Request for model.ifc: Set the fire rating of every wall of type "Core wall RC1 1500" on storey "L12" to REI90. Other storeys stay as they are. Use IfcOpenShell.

First a look at what the model holds.

```python
import ifcopenshell
import ifcopenshell.util.element

model = ifcopenshell.open("model.ifc")
print(model.schema)
storey = next(s for s in model.by_type("IfcBuildingStorey") if s.Name == "L12")
walls = [e for e in ifcopenshell.util.element.get_decomposition(storey) if e.is_a("IfcWall")]
seen = {}
for e in walls:
    element_type = ifcopenshell.util.element.get_type(e)
    key = (element_type.Name if element_type != e and element_type else None, ifcopenshell.util.element.get_pset(e, "Pset_WallCommon", "FireRating"))
    seen[key] = seen.get(key, 0) + 1
for (name, value), count in sorted(seen.items(), key=str):
    print(count, "x", name, "|", value)
```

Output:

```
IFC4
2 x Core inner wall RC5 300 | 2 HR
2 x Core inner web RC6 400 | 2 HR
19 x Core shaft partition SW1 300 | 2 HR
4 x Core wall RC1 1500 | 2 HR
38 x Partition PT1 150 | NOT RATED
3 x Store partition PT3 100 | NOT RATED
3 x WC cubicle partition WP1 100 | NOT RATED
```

```python
import ifcopenshell
import ifcopenshell.api.pset
import ifcopenshell.util.element

model = ifcopenshell.open("model.ifc")

storey = next(s for s in model.by_type("IfcBuildingStorey") if s.Name == "L12")
walls = [e for e in ifcopenshell.util.element.get_decomposition(storey) if e.is_a("IfcWall")]

count = 0
for e in walls:
    element_type = ifcopenshell.util.element.get_type(e)
    if element_type in (None, e) or element_type.Name != "Core wall RC1 1500":
        continue
    # add_pset returns the element's existing set when there is one.
    pset = ifcopenshell.api.pset.add_pset(model, product=e, name="Pset_WallCommon")
    ifcopenshell.api.pset.edit_pset(model, pset=pset, properties={"FireRating": "REI90"})
    count += 1

print(count, "walls updated")

model.write("model_rev.ifc")
```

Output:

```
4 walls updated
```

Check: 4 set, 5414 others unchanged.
